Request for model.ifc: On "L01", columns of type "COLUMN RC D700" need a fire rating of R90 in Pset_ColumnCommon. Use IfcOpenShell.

First a look at what the model holds.

```python
import ifcopenshell
import ifcopenshell.util.element

model = ifcopenshell.open("model.ifc")
print(model.schema)
storey = next(s for s in model.by_type("IfcBuildingStorey") if s.Name == "L01")
columns = [e for e in ifcopenshell.util.element.get_decomposition(storey) if e.is_a("IfcColumn")]
seen = {}
for e in columns:
    element_type = ifcopenshell.util.element.get_type(e)
    key = (element_type.Name if element_type != e and element_type else None, ifcopenshell.util.element.get_pset(e, "Pset_ColumnCommon", "FireRating"))
    seen[key] = seen.get(key, 0) + 1
for (name, value), count in sorted(seen.items(), key=str):
    print(count, "x", name, "|", value)
```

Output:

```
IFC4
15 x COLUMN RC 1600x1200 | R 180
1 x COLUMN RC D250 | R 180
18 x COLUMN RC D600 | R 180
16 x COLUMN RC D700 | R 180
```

```python
import ifcopenshell
import ifcopenshell.api.pset
import ifcopenshell.util.element

model = ifcopenshell.open("model.ifc")

storey = next(s for s in model.by_type("IfcBuildingStorey") if s.Name == "L01")
columns = [e for e in ifcopenshell.util.element.get_decomposition(storey) if e.is_a("IfcColumn")]

count = 0
for e in columns:
    element_type = ifcopenshell.util.element.get_type(e)
    if element_type in (None, e) or element_type.Name != "COLUMN RC D700":
        continue
    # add_pset returns the element's existing set when there is one.
    pset = ifcopenshell.api.pset.add_pset(model, product=e, name="Pset_ColumnCommon")
    ifcopenshell.api.pset.edit_pset(model, pset=pset, properties={"FireRating": "R90"})
    count += 1

print(count, "columns updated")

model.write("model-out.ifc")
```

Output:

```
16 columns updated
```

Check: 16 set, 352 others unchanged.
